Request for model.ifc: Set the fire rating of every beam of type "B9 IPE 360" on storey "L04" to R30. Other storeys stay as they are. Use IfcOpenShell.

First a look at what the model holds.

```python
import ifcopenshell
import ifcopenshell.util.element

model = ifcopenshell.open("model.ifc")
print(model.schema)
storey = next(s for s in model.by_type("IfcBuildingStorey") if s.Name == "L04")
beams = [e for e in ifcopenshell.util.element.get_decomposition(storey) if e.is_a("IfcBeam")]
seen = {}
for e in beams:
    element_type = ifcopenshell.util.element.get_type(e)
    key = (element_type.Name if element_type != e and element_type else None, ifcopenshell.util.element.get_pset(e, "Pset_BeamCommon", "FireRating"))
    seen[key] = seen.get(key, 0) + 1
for (name, value), count in sorted(seen.items(), key=str):
    print(count, "x", name, "|", value)
```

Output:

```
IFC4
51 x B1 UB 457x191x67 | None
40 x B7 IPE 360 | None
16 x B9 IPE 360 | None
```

```python
import ifcopenshell
import ifcopenshell.api.pset
import ifcopenshell.util.element

model = ifcopenshell.open("model.ifc")

storey = next(s for s in model.by_type("IfcBuildingStorey") if s.Name == "L04")
beams = [e for e in ifcopenshell.util.element.get_decomposition(storey) if e.is_a("IfcBeam")]

count = 0
for e in beams:
    element_type = ifcopenshell.util.element.get_type(e)
    if element_type in (None, e) or element_type.Name != "B9 IPE 360":
        continue
    # add_pset returns the element's existing set when there is one.
    pset = ifcopenshell.api.pset.add_pset(model, product=e, name="Pset_BeamCommon")
    ifcopenshell.api.pset.edit_pset(model, pset=pset, properties={"FireRating": "R30"})
    count += 1

print(count, "beams updated")

model.write("model_edited.ifc")
```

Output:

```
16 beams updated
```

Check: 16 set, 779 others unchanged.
